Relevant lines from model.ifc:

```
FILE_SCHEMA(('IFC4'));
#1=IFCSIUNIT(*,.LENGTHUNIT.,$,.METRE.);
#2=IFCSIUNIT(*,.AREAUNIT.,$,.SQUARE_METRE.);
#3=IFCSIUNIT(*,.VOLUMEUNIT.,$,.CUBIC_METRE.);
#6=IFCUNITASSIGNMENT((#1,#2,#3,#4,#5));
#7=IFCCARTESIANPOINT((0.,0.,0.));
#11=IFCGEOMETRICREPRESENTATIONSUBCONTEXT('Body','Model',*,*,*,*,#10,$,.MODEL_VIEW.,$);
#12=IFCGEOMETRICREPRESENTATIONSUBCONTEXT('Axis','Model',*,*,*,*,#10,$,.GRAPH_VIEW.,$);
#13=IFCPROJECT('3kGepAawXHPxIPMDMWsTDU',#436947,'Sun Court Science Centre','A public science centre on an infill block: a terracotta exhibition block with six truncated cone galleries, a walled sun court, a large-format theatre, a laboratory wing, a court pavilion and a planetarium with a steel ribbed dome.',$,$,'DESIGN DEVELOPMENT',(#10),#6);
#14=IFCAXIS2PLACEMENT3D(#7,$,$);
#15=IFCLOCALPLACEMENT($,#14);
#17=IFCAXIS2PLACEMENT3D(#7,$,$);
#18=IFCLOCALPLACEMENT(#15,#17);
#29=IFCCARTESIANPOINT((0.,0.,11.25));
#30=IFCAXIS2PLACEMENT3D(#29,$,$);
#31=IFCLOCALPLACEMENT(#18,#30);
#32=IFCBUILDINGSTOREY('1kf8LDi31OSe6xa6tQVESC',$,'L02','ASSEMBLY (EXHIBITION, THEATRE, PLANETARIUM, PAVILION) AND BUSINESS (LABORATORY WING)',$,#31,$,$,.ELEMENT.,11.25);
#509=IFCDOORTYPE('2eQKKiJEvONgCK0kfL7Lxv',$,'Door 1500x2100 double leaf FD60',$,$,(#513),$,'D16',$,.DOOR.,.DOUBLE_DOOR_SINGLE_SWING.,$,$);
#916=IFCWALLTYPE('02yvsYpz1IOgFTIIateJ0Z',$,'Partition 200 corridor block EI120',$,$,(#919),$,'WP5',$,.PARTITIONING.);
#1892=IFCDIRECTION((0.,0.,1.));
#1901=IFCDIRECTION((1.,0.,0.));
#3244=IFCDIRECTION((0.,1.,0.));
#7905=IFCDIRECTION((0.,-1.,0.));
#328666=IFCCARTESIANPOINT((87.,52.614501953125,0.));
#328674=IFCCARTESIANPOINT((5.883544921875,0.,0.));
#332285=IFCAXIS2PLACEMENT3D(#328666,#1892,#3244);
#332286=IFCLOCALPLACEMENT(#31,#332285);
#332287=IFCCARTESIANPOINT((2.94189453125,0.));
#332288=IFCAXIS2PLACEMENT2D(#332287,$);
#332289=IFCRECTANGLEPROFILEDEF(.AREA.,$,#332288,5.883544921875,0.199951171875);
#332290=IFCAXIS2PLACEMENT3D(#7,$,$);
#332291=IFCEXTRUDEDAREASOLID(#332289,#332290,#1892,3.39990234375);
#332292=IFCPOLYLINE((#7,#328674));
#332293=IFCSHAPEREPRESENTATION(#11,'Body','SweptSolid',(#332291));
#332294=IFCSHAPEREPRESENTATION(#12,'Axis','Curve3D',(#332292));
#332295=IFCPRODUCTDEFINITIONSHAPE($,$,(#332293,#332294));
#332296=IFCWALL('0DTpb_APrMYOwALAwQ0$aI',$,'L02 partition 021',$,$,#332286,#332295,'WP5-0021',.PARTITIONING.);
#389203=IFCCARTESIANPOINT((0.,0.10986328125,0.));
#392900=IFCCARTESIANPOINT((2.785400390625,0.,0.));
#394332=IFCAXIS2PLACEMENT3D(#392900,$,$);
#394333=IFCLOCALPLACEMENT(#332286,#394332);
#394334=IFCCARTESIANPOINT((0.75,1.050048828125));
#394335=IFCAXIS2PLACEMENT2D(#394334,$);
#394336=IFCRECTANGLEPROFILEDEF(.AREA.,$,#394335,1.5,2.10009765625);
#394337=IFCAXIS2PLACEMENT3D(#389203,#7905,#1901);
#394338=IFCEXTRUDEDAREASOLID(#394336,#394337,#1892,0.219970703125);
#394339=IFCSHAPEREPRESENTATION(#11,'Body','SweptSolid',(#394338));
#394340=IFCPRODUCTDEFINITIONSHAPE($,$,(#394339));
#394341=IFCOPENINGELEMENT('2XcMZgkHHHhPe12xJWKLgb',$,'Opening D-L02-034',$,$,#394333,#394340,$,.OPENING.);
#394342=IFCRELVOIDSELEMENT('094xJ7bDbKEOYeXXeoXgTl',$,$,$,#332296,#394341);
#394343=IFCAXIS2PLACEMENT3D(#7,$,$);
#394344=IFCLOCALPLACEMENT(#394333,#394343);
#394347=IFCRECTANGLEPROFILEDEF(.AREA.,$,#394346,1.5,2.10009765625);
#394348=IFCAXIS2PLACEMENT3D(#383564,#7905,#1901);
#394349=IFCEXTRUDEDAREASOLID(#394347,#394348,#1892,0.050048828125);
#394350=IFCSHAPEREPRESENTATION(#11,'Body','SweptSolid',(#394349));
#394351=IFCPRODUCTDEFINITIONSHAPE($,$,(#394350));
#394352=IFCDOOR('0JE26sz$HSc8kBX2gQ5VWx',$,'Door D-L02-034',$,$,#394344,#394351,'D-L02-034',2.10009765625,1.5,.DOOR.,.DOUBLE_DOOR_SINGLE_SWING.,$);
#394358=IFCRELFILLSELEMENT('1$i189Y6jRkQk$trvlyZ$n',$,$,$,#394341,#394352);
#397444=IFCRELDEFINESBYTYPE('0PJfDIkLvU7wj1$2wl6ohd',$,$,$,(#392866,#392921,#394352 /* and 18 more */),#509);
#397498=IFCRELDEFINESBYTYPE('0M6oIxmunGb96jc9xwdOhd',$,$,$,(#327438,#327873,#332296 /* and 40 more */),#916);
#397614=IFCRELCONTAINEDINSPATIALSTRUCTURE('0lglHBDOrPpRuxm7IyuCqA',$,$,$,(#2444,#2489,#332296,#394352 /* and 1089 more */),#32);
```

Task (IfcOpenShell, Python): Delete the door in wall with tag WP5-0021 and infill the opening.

```python
import ifcopenshell
import ifcopenshell.api.feature
import ifcopenshell.api.root
import ifcopenshell.geom
import ifcopenshell.util.shape

model = ifcopenshell.open("model.ifc")
settings = ifcopenshell.geom.settings()


def volume(element):
    """Net volume in cubic metres, openings subtracted."""
    shape = ifcopenshell.geom.create_shape(settings, element)
    return ifcopenshell.util.shape.get_volume(shape.geometry)


door = model.by_guid("0JE26sz$HSc8kBX2gQ5VWx")
opening = door.FillsVoids[0].RelatingOpeningElement
wall = opening.VoidsElements[0].RelatingBuildingElement
before = volume(wall)

ifcopenshell.api.root.remove_product(model, product=door)
ifcopenshell.api.feature.remove_feature(model, feature=opening)

after = volume(wall)

print(f"wall volume {before:.3f} -> {after:.3f} m3")

model.write("model_v2.ifc")
```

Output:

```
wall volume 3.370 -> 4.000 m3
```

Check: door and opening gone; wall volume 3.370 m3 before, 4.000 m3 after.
